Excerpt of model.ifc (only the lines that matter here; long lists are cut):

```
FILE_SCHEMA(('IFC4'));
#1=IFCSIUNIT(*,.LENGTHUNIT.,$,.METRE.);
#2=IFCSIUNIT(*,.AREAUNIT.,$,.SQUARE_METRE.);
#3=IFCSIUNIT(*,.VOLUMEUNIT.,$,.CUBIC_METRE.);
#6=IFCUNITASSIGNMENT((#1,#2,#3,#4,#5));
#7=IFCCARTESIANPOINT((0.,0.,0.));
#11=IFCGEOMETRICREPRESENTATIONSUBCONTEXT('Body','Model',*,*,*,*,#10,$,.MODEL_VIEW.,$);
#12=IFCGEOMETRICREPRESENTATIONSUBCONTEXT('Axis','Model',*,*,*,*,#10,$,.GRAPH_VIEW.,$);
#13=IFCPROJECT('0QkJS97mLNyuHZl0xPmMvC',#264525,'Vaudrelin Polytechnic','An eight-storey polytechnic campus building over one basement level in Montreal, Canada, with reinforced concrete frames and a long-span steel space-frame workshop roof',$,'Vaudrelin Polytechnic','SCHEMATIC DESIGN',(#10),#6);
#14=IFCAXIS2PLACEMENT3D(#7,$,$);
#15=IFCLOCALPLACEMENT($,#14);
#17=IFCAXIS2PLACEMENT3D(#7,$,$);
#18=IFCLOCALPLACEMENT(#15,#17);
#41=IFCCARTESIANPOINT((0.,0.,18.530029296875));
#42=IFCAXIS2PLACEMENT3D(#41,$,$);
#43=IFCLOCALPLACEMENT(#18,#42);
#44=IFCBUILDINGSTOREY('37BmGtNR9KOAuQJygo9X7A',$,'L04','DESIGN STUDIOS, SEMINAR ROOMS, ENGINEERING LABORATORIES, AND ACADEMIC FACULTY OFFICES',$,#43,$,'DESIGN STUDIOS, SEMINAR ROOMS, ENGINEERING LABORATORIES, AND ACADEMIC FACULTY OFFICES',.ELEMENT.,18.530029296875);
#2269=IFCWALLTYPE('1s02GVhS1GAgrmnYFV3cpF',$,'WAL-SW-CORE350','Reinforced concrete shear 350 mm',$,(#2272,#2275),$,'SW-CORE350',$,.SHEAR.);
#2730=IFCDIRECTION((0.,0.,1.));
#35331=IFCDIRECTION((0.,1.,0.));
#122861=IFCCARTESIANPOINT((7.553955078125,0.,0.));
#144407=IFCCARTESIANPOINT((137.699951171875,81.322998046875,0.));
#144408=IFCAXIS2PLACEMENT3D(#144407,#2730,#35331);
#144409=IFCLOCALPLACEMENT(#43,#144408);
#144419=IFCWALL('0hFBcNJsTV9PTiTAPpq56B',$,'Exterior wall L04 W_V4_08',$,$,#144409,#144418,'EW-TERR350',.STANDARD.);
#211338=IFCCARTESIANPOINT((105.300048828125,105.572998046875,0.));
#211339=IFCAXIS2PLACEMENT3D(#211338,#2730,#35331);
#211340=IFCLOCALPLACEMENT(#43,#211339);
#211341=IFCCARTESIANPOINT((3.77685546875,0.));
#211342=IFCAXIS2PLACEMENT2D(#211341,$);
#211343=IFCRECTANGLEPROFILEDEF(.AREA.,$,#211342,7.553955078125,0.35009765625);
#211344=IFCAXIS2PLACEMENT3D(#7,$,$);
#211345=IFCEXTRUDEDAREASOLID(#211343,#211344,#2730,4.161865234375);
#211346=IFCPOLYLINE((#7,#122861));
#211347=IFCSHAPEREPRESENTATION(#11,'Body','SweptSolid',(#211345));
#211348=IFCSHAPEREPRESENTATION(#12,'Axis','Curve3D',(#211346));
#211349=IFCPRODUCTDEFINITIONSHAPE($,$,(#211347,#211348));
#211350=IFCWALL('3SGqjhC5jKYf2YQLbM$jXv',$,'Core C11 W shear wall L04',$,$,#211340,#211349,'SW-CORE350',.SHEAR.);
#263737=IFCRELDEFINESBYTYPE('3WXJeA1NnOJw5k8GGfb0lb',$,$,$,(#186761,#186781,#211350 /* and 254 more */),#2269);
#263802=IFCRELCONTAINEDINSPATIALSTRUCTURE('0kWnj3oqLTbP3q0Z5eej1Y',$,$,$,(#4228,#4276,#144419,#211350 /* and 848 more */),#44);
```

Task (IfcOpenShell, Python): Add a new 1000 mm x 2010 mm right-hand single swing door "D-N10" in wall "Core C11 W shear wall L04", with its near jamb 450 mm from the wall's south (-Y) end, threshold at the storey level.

```python
import numpy as np
import ifcopenshell
import ifcopenshell.api.feature
import ifcopenshell.api.geometry
import ifcopenshell.api.root
import ifcopenshell.api.spatial
import ifcopenshell.geom
import ifcopenshell.util.element
import ifcopenshell.util.placement
import ifcopenshell.util.representation
import ifcopenshell.util.shape
import ifcopenshell.util.unit

model = ifcopenshell.open("model.ifc")
unit_scale = ifcopenshell.util.unit.calculate_unit_scale(model)
settings = ifcopenshell.geom.settings()


def volume(element):
    """Net volume in cubic metres, openings subtracted."""
    shape = ifcopenshell.geom.create_shape(settings, element)
    return ifcopenshell.util.shape.get_volume(shape.geometry)


wall = model.by_id(211350)
storey = ifcopenshell.util.element.get_container(wall, ifc_class="IfcBuildingStorey")
context = ifcopenshell.util.representation.get_context(model, "Model", "Body", "MODEL_VIEW")
before = volume(wall)

width, height, from_end, sill = 1, 2.01, 0.45, 0.0  # metres

# The wall runs along its own X axis, and the end named is its -X end.
wall_shape = ifcopenshell.geom.create_shape(settings, wall)
x, y, z = ifcopenshell.util.shape.get_vertices(wall_shape.geometry).T
start = x.min() + from_end
face, thickness = float(y.min()), float(y.max() - y.min())
wall_matrix = ifcopenshell.util.placement.get_local_placement(wall.ObjectPlacement)
level = ifcopenshell.util.placement.get_local_placement(storey.ObjectPlacement)[2, 3]


def in_wall(x, y):
    """Placement at x, y metres in the wall's axes, at sill height."""
    matrix = wall_matrix.copy()
    matrix[:, 3] = wall_matrix @ np.array([x / unit_scale, y / unit_scale, 0.0, 1.0])
    matrix[2, 3] = level + sill / unit_scale
    return matrix


# Opening: a box that overshoots both wall faces by 50 mm.
opening = ifcopenshell.api.root.create_entity(model, ifc_class="IfcOpeningElement", predefined_type="OPENING")
box = ifcopenshell.api.geometry.add_wall_representation(
    model, context=context, length=width, height=height, thickness=thickness + 0.1
)
ifcopenshell.api.geometry.assign_representation(model, product=opening, representation=box)
ifcopenshell.api.geometry.edit_object_placement(model, product=opening, matrix=in_wall(start, face - 0.05), is_si=False)
ifcopenshell.api.feature.add_feature(model, feature=opening, element=wall)

door = ifcopenshell.api.root.create_entity(model, ifc_class="IfcDoor", name="D-N10", predefined_type="DOOR")
door.OverallWidth, door.OverallHeight = width / unit_scale, height / unit_scale
door.OperationType = "SINGLE_SWING_RIGHT"
body = ifcopenshell.api.geometry.add_door_representation(
    model,
    context=context,
    overall_width=door.OverallWidth,
    overall_height=door.OverallHeight,
    operation_type="SINGLE_SWING_RIGHT",
    lining_properties={"LiningDepth": thickness / unit_scale, "ThresholdDepth": thickness / unit_scale},
)
ifcopenshell.api.geometry.assign_representation(model, product=door, representation=body)
ifcopenshell.api.spatial.assign_container(model, products=[door], relating_structure=storey)
ifcopenshell.api.feature.add_filling(model, opening=opening, element=door)

# The lining spans the wall, so the door starts at the wall face.
ifcopenshell.api.geometry.edit_object_placement(model, product=door, matrix=in_wall(start, face), is_si=False)

after = volume(wall)

print(f"wall volume {before:.3f} -> {after:.3f} m3")

model.write("model_v2.ifc")
```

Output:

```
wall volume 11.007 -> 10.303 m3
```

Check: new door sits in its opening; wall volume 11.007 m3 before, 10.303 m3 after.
